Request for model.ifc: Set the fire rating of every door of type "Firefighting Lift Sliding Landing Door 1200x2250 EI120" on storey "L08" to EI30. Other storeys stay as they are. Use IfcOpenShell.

First a look at what the model holds.

```python
import ifcopenshell
import ifcopenshell.util.element

model = ifcopenshell.open("model.ifc")
print(model.schema)
storey = next(s for s in model.by_type("IfcBuildingStorey") if s.Name == "L08")
doors = [e for e in ifcopenshell.util.element.get_decomposition(storey) if e.is_a("IfcDoor")]
seen = {}
for e in doors:
    element_type = ifcopenshell.util.element.get_type(e)
    key = (element_type.Name if element_type != e and element_type else None, ifcopenshell.util.element.get_pset(e, "Pset_DoorCommon", "FireRating"))
    seen[key] = seen.get(key, 0) + 1
for (name, value), count in sorted(seen.items(), key=str):
    print(count, "x", name, "|", value)
```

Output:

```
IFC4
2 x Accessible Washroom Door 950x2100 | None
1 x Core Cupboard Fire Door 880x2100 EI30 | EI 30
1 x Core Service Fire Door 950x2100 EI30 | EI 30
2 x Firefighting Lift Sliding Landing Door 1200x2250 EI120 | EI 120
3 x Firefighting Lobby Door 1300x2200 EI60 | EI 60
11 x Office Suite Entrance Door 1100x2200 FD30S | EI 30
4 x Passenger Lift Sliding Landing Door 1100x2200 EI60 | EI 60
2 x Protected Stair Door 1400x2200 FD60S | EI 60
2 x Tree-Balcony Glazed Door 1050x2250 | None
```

```python
import ifcopenshell
import ifcopenshell.api.pset
import ifcopenshell.util.element

model = ifcopenshell.open("model.ifc")

storey = next(s for s in model.by_type("IfcBuildingStorey") if s.Name == "L08")
doors = [e for e in ifcopenshell.util.element.get_decomposition(storey) if e.is_a("IfcDoor")]

count = 0
for e in doors:
    element_type = ifcopenshell.util.element.get_type(e)
    if element_type in (None, e) or element_type.Name != "Firefighting Lift Sliding Landing Door 1200x2250 EI120":
        continue
    # add_pset returns the element's existing set when there is one.
    pset = ifcopenshell.api.pset.add_pset(model, product=e, name="Pset_DoorCommon")
    ifcopenshell.api.pset.edit_pset(model, pset=pset, properties={"FireRating": "EI30"})
    count += 1

print(count, "doors updated")

model.write("model_v2.ifc")
```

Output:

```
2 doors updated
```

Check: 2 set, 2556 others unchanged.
